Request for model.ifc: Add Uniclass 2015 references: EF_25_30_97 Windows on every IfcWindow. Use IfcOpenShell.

First a look at what the model holds.

```python
import ifcopenshell

model = ifcopenshell.open("model.ifc")
print(model.schema)
print("classifications:", [c.Name for c in model.by_type("IfcClassification")])
for ifc_class in ("IfcDoor", "IfcRoof", "IfcStair", "IfcWall", "IfcWindow"):
    print(ifc_class, len(model.by_type(ifc_class)))
```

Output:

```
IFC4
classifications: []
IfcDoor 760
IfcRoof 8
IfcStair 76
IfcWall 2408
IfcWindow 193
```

```python
import ifcopenshell
import ifcopenshell.api.classification

model = ifcopenshell.open("model.ifc")

system = ifcopenshell.api.classification.add_classification(model, classification="Uniclass 2015")

codes = {
    "IfcWindow": ("EF_25_30_97", "Windows"),
}
for ifc_class, (code, name) in codes.items():
    products = model.by_type(ifc_class)
    ifcopenshell.api.classification.add_reference(
        model, products=products, classification=system, identification=code, name=name
    )
    print(code, len(products))

model.write("model_v2.ifc")
```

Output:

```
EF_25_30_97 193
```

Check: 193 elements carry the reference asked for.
